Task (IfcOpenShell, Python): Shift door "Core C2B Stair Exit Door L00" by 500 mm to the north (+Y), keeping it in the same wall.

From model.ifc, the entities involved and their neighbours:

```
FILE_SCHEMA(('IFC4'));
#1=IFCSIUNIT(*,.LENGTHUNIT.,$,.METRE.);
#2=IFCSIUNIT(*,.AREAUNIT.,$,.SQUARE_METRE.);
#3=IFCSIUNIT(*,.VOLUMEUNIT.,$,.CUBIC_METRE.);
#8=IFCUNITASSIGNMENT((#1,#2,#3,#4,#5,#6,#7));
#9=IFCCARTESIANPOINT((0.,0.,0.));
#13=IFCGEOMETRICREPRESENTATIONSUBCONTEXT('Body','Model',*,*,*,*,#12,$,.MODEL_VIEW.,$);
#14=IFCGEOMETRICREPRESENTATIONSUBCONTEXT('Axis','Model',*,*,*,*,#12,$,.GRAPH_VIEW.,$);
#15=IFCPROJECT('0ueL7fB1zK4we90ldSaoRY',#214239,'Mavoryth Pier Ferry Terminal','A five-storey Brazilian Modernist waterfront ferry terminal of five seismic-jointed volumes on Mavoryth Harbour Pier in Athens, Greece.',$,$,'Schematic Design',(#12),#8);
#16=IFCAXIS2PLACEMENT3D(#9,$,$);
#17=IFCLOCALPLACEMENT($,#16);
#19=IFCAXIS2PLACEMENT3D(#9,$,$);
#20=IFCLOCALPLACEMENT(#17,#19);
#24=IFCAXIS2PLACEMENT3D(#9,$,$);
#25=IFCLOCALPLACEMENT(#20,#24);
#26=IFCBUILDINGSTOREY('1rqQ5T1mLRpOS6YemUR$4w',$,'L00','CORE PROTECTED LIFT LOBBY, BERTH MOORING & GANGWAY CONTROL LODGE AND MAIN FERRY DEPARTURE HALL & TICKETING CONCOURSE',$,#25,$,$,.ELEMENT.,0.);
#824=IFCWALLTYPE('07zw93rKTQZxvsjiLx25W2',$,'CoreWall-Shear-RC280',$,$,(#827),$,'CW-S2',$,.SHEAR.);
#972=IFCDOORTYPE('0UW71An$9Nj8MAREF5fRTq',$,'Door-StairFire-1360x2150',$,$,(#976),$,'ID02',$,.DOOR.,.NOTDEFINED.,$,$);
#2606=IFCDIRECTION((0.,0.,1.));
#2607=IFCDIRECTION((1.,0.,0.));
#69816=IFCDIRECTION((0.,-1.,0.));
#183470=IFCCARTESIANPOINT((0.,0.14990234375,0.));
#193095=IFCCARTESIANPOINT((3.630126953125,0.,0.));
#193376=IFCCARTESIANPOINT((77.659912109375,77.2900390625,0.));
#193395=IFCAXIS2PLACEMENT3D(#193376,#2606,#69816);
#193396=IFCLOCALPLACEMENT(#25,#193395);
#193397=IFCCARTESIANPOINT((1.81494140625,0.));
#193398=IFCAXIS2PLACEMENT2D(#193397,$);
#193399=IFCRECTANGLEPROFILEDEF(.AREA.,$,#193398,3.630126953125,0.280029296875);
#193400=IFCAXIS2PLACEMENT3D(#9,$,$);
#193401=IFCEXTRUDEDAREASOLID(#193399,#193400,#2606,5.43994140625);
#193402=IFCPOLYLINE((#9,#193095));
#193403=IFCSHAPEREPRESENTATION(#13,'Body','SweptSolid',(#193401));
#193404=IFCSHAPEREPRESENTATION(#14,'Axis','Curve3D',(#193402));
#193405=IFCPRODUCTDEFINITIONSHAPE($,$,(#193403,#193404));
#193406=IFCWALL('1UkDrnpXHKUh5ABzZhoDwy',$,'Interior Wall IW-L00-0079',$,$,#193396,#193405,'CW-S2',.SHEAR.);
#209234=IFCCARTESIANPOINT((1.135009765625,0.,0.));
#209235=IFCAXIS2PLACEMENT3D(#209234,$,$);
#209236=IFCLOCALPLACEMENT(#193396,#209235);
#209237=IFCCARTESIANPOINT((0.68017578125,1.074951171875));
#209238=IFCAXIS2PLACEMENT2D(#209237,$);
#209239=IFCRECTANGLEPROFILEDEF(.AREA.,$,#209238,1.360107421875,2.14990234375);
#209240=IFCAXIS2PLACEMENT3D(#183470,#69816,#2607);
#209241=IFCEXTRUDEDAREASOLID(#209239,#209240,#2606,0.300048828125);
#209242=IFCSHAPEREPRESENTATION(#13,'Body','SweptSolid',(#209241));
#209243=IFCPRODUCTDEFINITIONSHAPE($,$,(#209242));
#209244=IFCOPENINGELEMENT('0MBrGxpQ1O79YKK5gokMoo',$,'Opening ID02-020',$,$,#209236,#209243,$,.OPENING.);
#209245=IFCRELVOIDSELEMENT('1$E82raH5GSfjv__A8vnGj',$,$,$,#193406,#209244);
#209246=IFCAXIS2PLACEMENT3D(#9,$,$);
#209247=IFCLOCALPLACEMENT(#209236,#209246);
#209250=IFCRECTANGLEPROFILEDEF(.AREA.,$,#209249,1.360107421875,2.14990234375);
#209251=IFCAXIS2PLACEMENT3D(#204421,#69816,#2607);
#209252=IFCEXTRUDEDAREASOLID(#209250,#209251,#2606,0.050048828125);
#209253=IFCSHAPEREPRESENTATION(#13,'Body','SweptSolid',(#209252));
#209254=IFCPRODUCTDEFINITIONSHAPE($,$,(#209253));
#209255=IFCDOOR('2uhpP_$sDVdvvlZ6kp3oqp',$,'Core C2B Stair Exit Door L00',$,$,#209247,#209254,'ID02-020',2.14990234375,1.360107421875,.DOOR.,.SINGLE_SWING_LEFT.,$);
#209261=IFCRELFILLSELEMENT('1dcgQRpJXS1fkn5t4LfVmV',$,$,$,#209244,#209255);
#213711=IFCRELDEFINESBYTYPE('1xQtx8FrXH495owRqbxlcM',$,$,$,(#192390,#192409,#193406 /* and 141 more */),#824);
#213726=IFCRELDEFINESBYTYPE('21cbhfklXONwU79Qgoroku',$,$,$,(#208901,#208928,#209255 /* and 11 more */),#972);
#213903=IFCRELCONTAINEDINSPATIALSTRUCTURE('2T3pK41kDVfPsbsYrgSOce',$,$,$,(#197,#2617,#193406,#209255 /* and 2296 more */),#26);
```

```python
import ifcopenshell
import ifcopenshell.api.geometry
import ifcopenshell.util.placement
import ifcopenshell.util.unit

model = ifcopenshell.open("model.ifc")
unit_scale = ifcopenshell.util.unit.calculate_unit_scale(model)

door = model.by_guid("2uhpP_$sDVdvvlZ6kp3oqp")
opening = door.FillsVoids[0].RelatingOpeningElement
wall = opening.VoidsElements[0].RelatingBuildingElement

wall_matrix = ifcopenshell.util.placement.get_local_placement(wall.ObjectPlacement)
shift = wall_matrix[:3, 0] * -0.5 / unit_scale
before = ifcopenshell.util.placement.get_local_placement(door.ObjectPlacement)[:3, 3].copy()

# The door is placed relative to its opening, so it follows when the opening moves.
matrix = ifcopenshell.util.placement.get_local_placement(opening.ObjectPlacement)
matrix[:3, 3] += shift
ifcopenshell.api.geometry.edit_object_placement(
    model, product=opening, matrix=matrix, is_si=False, should_transform_children=True
)

after = ifcopenshell.util.placement.get_local_placement(door.ObjectPlacement)[:3, 3]
print("door moved by", (after - before).round(3) + 0.0)

model.write("model_rev.ifc")
```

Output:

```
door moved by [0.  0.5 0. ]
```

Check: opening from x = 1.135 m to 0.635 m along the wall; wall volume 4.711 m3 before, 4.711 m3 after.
